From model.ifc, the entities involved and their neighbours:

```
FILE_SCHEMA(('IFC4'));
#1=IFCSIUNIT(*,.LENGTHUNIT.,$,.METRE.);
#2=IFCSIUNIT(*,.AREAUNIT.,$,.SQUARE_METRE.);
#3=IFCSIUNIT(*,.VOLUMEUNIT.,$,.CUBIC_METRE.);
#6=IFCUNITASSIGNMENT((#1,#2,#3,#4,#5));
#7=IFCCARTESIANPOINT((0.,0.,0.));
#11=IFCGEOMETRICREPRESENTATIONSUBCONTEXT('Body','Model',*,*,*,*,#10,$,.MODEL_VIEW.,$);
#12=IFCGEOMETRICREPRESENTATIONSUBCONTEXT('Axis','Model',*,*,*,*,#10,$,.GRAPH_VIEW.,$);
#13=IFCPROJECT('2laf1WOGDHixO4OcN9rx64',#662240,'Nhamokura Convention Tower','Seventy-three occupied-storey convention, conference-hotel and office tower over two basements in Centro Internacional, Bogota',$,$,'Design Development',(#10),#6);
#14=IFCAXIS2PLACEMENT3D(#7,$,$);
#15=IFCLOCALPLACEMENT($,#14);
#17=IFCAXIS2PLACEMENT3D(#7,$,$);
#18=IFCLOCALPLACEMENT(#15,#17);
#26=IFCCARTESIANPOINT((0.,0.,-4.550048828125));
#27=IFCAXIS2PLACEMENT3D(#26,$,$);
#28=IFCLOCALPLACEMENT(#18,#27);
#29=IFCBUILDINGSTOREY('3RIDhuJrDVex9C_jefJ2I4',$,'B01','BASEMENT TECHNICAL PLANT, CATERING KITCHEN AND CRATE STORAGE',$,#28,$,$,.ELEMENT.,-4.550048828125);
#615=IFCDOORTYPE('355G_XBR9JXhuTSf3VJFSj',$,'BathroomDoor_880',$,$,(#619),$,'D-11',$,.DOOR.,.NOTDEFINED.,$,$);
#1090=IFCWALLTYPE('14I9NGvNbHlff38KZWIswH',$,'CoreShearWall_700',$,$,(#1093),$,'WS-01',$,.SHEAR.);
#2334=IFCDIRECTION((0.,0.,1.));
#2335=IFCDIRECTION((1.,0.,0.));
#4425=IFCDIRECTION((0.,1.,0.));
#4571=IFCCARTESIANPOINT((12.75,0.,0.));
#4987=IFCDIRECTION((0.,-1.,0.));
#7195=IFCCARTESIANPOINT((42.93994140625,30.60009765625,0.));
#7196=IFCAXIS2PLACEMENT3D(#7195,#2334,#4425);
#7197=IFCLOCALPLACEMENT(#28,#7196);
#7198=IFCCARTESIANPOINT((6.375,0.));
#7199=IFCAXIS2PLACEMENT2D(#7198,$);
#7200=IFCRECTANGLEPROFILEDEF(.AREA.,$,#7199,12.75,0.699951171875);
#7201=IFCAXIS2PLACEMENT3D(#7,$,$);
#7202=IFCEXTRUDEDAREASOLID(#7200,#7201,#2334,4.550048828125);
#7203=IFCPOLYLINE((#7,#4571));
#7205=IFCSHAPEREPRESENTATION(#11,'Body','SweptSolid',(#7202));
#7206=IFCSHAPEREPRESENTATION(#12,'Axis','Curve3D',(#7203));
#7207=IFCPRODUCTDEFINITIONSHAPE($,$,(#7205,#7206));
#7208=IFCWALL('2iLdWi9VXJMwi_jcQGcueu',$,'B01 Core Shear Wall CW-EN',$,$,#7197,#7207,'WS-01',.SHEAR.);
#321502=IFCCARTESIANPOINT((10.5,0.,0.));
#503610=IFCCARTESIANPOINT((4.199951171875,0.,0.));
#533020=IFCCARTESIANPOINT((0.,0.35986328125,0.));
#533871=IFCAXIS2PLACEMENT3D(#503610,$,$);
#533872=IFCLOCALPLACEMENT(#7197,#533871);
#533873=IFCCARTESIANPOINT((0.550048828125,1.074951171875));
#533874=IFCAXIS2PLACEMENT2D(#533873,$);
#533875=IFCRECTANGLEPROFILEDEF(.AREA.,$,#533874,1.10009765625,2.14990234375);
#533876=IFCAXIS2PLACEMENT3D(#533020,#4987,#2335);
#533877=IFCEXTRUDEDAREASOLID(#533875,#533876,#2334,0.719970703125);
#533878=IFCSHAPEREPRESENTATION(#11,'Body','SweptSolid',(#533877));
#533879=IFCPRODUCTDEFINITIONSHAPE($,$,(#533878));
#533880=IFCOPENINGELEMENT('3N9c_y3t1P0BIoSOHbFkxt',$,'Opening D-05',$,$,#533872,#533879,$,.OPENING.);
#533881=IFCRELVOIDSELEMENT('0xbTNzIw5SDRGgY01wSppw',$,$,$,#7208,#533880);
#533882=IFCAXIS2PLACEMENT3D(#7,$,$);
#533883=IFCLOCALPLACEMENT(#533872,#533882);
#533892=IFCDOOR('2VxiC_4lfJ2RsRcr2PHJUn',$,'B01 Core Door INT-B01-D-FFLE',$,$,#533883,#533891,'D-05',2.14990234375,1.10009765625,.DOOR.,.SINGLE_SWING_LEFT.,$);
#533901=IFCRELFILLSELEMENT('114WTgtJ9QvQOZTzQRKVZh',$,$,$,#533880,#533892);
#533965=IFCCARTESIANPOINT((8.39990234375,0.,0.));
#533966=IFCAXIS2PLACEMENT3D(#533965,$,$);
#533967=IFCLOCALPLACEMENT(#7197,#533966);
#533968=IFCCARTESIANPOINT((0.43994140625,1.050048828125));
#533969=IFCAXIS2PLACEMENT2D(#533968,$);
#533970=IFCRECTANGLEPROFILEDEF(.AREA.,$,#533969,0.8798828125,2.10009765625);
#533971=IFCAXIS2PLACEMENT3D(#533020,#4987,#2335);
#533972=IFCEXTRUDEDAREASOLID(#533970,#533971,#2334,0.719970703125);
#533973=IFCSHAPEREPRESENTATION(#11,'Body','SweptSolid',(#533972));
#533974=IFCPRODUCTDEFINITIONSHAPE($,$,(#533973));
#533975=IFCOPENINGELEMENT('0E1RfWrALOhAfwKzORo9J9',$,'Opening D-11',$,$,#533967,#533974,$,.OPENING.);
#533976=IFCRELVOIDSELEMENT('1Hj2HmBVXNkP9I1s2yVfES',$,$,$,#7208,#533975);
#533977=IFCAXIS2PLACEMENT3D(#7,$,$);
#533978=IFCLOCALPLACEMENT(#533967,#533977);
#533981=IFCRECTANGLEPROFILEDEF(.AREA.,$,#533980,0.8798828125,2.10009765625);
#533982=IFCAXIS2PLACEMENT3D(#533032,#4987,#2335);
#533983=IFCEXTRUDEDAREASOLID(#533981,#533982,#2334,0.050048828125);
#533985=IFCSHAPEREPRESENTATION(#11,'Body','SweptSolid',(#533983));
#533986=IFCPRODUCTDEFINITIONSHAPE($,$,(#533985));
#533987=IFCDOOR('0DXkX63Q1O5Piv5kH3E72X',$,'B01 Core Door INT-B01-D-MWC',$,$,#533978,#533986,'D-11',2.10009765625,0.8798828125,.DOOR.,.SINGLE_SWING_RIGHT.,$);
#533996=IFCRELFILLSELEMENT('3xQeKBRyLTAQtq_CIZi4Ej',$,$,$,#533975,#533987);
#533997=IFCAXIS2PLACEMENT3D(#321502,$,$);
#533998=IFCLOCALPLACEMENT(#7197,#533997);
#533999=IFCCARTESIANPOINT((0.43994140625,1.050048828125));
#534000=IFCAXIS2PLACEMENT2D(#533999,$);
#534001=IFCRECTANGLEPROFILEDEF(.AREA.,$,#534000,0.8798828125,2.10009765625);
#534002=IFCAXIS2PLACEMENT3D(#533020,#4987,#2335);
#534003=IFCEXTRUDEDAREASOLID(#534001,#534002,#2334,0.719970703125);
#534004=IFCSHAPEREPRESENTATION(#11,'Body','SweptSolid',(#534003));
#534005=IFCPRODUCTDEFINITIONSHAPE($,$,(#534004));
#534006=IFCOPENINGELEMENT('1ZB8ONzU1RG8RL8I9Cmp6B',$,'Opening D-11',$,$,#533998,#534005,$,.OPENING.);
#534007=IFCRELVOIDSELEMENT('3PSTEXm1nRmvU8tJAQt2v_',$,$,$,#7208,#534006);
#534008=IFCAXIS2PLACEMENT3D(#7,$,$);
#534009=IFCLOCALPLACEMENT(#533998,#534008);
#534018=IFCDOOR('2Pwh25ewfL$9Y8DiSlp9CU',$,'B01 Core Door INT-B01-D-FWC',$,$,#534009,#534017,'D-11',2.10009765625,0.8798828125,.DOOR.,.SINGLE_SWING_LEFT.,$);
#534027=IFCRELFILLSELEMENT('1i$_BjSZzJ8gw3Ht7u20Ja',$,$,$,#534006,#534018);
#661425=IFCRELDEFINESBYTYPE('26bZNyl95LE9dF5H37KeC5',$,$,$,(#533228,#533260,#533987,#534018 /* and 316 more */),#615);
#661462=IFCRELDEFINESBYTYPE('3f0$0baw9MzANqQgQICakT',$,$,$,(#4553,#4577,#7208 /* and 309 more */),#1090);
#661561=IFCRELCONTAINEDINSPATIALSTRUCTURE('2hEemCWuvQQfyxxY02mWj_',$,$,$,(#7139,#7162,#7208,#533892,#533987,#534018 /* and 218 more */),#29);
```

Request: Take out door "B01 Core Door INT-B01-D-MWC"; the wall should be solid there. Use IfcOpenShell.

```python
import ifcopenshell
import ifcopenshell.api.feature
import ifcopenshell.api.root
import ifcopenshell.geom
import ifcopenshell.util.shape

model = ifcopenshell.open("model.ifc")
settings = ifcopenshell.geom.settings()


def volume(element):
    """Net volume in cubic metres, openings subtracted."""
    shape = ifcopenshell.geom.create_shape(settings, element)
    return ifcopenshell.util.shape.get_volume(shape.geometry)


door = model.by_guid("0DXkX63Q1O5Piv5kH3E72X")
opening = door.FillsVoids[0].RelatingOpeningElement
wall = opening.VoidsElements[0].RelatingBuildingElement
before = volume(wall)

ifcopenshell.api.root.remove_product(model, product=door)
ifcopenshell.api.feature.remove_feature(model, feature=opening)

after = volume(wall)

print(f"wall volume {before:.3f} -> {after:.3f} m3")

model.write("model-out.ifc")
```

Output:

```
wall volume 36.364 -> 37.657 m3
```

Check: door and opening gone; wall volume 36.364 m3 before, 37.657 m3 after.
